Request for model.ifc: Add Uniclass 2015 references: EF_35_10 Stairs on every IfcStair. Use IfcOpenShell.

First a look at what the model holds.

```python
import ifcopenshell

model = ifcopenshell.open("model.ifc")
print(model.schema)
print("classifications:", [c.Name for c in model.by_type("IfcClassification")])
for ifc_class in ("IfcDoor", "IfcRoof", "IfcStair", "IfcWall", "IfcWindow"):
    print(ifc_class, len(model.by_type(ifc_class)))
```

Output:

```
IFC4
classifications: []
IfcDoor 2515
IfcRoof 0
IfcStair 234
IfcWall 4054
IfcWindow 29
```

```python
import ifcopenshell
import ifcopenshell.api.classification

model = ifcopenshell.open("model.ifc")

system = ifcopenshell.api.classification.add_classification(model, classification="Uniclass 2015")

codes = {
    "IfcStair": ("EF_35_10", "Stairs"),
}
for ifc_class, (code, name) in codes.items():
    products = model.by_type(ifc_class)
    ifcopenshell.api.classification.add_reference(
        model, products=products, classification=system, identification=code, name=name
    )
    print(code, len(products))

model.write("model_updated.ifc")
```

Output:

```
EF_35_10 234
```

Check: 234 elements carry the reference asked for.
